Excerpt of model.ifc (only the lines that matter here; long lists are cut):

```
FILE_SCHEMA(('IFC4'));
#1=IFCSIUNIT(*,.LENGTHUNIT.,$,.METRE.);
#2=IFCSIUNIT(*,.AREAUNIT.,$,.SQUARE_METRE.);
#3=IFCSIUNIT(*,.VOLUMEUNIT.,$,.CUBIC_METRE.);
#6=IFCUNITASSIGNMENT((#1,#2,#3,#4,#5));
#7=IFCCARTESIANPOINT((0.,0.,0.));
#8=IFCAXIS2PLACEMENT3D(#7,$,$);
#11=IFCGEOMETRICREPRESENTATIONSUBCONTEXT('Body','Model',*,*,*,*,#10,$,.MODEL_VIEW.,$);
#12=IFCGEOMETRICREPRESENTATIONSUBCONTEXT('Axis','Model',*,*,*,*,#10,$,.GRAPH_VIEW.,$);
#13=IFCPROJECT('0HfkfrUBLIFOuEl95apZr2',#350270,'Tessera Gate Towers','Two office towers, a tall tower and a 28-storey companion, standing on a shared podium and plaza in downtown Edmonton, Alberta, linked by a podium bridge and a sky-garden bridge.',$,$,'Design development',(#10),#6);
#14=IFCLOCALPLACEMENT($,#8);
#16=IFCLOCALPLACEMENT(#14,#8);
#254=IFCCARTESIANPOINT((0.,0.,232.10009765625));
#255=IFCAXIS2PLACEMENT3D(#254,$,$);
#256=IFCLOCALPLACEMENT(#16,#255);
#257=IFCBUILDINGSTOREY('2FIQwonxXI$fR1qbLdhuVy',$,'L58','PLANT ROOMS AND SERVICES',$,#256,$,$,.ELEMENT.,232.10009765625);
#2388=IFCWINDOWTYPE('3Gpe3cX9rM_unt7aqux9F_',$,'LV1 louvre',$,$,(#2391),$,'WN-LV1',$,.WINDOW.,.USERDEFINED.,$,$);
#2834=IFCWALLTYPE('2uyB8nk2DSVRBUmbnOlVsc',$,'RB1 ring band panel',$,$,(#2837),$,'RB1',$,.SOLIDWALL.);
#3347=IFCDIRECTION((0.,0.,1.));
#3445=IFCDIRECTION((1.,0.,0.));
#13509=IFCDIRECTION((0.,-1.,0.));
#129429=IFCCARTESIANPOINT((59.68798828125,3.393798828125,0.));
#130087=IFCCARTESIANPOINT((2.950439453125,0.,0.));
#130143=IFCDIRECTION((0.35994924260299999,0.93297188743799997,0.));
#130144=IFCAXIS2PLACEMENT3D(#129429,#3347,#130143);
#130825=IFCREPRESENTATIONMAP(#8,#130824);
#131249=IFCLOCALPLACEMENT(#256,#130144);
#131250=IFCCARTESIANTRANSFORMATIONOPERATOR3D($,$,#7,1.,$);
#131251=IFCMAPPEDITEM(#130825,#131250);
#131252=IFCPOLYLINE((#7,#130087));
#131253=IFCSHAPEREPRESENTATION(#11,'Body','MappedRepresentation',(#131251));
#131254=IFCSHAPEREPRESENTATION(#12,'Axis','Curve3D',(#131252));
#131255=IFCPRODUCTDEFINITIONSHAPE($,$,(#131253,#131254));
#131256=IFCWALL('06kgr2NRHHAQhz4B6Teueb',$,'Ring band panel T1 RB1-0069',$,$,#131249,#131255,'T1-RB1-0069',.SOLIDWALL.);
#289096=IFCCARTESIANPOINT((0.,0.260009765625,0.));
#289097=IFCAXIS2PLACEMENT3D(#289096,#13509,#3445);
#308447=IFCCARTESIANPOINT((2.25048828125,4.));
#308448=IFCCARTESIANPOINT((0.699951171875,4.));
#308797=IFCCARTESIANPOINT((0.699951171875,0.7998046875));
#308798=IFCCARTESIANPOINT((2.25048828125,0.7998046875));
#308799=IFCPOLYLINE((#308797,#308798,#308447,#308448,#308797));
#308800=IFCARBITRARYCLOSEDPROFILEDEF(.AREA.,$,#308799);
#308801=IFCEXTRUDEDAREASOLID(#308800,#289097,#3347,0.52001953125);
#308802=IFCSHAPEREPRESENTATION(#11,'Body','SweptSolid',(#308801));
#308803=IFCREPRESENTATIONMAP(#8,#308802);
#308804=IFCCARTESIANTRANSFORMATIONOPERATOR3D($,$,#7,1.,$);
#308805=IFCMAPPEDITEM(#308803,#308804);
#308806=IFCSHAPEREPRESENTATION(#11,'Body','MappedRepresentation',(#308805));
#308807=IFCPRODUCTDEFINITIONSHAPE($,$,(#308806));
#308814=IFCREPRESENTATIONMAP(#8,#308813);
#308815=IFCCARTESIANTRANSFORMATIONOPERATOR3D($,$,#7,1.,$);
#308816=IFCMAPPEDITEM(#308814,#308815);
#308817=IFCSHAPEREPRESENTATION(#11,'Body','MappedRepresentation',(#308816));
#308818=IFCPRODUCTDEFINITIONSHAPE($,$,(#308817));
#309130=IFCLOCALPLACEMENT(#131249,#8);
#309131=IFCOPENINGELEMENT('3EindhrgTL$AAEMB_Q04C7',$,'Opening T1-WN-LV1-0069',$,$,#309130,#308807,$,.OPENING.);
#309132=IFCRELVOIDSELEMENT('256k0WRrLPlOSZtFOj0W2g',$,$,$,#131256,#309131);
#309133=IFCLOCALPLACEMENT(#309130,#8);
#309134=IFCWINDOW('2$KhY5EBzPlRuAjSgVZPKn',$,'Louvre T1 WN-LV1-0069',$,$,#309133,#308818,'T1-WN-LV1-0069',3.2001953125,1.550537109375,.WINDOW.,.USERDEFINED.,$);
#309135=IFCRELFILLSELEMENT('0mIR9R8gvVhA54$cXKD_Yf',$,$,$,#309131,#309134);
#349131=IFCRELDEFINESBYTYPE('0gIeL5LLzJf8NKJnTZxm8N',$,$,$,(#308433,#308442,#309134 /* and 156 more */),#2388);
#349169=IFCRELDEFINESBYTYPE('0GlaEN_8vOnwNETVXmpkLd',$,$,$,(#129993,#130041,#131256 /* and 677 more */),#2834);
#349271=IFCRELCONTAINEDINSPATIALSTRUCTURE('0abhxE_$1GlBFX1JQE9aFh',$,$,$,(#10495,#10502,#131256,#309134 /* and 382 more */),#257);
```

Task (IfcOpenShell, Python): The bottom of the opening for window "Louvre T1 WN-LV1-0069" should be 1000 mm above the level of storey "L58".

```python
import numpy as np
import ifcopenshell
import ifcopenshell.api.geometry
import ifcopenshell.geom
import ifcopenshell.util.element
import ifcopenshell.util.placement
import ifcopenshell.util.shape
import ifcopenshell.util.unit

model = ifcopenshell.open("model.ifc")
unit_scale = ifcopenshell.util.unit.calculate_unit_scale(model)

window = model.by_guid("2$KhY5EBzPlRuAjSgVZPKn")
opening = window.FillsVoids[0].RelatingOpeningElement
storey = ifcopenshell.util.element.get_container(window, ifc_class="IfcBuildingStorey")
level = ifcopenshell.util.placement.get_local_placement(storey.ObjectPlacement)[2, 3]

# The opening's origin need not be at the sill, so measure its lowest point.
shape = ifcopenshell.geom.create_shape(ifcopenshell.geom.settings(), opening)
bottom = ifcopenshell.util.shape.get_shape_bottom_elevation(shape, shape.geometry) / unit_scale
dz = level + 1 / unit_scale - bottom

shift = np.array([0.0, 0.0, dz])
# The window is placed relative to its opening, so it follows when the opening moves.
matrix = ifcopenshell.util.placement.get_local_placement(opening.ObjectPlacement)
matrix[:3, 3] += shift
ifcopenshell.api.geometry.edit_object_placement(
    model, product=opening, matrix=matrix, is_si=False, should_transform_children=True
)

print(f"moved by {dz * unit_scale:+.3f} m")

model.write("model_v2.ifc")
```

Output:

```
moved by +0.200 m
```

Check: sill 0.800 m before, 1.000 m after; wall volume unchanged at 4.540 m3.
